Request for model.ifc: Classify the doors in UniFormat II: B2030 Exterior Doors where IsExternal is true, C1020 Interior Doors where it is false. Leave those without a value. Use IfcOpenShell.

First a look at what the model holds.

```python
import ifcopenshell
import ifcopenshell.util.element

model = ifcopenshell.open("model.ifc")
print(model.schema)
print("classifications:", [c.Name for c in model.by_type("IfcClassification")])
values = [ifcopenshell.util.element.get_pset(e, "Pset_DoorCommon", "IsExternal") for e in model.by_type("IfcDoor")]
for value in (True, False, None):
    print("IsExternal", value, values.count(value))
```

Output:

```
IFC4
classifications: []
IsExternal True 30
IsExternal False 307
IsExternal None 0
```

```python
import ifcopenshell
import ifcopenshell.api.classification
import ifcopenshell.util.element

model = ifcopenshell.open("model.ifc")

system = ifcopenshell.api.classification.add_classification(model, classification="UniFormat II")

doors = model.by_type("IfcDoor")
external = {e: ifcopenshell.util.element.get_pset(e, "Pset_DoorCommon", "IsExternal") for e in doors}
for flag, code, name in ((True, "B2030", "Exterior Doors"), (False, "C1020", "Interior Doors")):
    products = [e for e in doors if external[e] is flag]
    ifcopenshell.api.classification.add_reference(
        model, products=products, classification=system, identification=code, name=name
    )
    print(code, len(products))

model.write("model_edited.ifc")
```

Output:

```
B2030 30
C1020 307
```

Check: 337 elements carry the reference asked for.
